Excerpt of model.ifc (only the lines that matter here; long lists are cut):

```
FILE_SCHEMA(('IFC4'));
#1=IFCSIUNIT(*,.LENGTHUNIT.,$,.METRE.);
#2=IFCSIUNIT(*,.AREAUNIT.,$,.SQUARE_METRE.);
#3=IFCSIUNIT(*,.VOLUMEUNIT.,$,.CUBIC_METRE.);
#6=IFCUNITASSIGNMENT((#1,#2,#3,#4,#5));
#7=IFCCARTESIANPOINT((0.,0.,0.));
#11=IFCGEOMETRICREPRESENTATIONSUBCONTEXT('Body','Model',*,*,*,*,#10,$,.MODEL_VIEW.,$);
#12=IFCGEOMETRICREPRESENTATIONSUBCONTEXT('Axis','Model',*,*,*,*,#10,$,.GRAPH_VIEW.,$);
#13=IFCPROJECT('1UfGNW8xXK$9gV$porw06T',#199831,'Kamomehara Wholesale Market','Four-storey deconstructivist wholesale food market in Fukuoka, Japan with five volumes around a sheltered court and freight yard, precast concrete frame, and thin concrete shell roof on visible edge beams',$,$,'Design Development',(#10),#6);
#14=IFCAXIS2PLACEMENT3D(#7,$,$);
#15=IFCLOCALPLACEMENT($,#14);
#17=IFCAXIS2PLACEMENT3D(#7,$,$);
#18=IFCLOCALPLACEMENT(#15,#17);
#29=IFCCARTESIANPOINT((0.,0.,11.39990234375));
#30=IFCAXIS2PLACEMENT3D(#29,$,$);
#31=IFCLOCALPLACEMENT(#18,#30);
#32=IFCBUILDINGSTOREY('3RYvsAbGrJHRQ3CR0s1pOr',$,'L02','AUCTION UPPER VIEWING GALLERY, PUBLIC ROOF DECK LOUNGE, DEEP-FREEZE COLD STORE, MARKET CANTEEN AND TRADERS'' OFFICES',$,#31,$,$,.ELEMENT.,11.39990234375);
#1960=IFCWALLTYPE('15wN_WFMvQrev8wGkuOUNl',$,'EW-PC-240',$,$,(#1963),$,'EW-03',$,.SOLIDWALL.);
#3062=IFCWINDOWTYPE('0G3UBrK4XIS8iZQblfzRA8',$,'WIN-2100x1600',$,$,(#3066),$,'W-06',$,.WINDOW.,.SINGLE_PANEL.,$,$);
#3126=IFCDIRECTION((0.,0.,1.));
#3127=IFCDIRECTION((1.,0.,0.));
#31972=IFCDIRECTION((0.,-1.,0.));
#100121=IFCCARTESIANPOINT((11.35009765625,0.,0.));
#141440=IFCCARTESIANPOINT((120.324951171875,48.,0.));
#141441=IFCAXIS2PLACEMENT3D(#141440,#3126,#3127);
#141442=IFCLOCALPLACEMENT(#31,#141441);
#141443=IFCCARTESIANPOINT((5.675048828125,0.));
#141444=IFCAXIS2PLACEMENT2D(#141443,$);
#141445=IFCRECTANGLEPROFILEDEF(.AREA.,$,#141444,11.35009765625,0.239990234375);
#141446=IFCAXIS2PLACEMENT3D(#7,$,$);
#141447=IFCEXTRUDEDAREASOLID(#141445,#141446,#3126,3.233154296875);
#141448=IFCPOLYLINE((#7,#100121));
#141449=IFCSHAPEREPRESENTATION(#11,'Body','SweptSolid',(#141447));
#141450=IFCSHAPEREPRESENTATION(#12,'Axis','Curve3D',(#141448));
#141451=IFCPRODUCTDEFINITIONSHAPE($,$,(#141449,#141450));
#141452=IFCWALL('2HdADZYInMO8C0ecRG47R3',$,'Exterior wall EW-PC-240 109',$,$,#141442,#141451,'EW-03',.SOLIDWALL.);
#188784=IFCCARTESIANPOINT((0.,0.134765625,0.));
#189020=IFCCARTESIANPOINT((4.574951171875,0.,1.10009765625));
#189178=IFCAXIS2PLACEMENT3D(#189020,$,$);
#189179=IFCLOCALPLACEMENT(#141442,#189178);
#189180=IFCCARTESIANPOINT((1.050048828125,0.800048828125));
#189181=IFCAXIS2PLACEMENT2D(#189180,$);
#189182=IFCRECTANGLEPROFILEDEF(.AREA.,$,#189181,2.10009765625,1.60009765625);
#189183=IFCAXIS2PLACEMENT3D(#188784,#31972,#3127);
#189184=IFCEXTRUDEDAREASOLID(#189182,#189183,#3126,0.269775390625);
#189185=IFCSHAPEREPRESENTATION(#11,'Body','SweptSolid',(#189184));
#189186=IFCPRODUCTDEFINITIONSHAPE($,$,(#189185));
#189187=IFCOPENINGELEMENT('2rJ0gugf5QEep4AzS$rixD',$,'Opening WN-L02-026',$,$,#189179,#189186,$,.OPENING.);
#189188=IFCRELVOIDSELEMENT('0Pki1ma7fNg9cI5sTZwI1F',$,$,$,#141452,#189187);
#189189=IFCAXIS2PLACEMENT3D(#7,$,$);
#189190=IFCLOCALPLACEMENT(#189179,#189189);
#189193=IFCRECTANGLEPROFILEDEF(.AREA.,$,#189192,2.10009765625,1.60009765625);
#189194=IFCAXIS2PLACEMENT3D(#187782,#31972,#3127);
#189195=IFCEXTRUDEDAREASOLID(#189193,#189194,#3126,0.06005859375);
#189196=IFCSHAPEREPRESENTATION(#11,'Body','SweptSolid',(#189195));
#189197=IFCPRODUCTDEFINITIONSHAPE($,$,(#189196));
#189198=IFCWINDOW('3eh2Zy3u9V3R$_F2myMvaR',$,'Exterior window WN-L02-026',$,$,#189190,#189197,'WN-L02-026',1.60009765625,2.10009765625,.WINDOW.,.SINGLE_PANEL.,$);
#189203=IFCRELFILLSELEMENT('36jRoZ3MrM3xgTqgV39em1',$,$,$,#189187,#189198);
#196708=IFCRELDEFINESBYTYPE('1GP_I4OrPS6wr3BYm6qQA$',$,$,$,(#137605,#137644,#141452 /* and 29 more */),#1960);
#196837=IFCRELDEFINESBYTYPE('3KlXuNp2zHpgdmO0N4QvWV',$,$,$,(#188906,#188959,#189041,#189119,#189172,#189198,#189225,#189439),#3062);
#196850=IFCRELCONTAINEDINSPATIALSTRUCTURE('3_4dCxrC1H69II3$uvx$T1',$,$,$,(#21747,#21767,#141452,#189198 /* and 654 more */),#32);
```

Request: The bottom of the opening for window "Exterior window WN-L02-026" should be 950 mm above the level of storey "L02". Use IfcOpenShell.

```python
import numpy as np
import ifcopenshell
import ifcopenshell.api.geometry
import ifcopenshell.geom
import ifcopenshell.util.element
import ifcopenshell.util.placement
import ifcopenshell.util.shape
import ifcopenshell.util.unit

model = ifcopenshell.open("model.ifc")
unit_scale = ifcopenshell.util.unit.calculate_unit_scale(model)

window = model.by_guid("3eh2Zy3u9V3R$_F2myMvaR")
opening = window.FillsVoids[0].RelatingOpeningElement
storey = ifcopenshell.util.element.get_container(window, ifc_class="IfcBuildingStorey")
level = ifcopenshell.util.placement.get_local_placement(storey.ObjectPlacement)[2, 3]

# The opening's origin need not be at the sill, so measure its lowest point.
shape = ifcopenshell.geom.create_shape(ifcopenshell.geom.settings(), opening)
bottom = ifcopenshell.util.shape.get_shape_bottom_elevation(shape, shape.geometry) / unit_scale
dz = level + 0.95 - bottom

shift = np.array([0.0, 0.0, dz])
# The window is placed relative to its opening, so it follows when the opening moves.
matrix = ifcopenshell.util.placement.get_local_placement(opening.ObjectPlacement)
matrix[:3, 3] += shift
ifcopenshell.api.geometry.edit_object_placement(
    model, product=opening, matrix=matrix, is_si=False, should_transform_children=True
)

print(f"moved by {dz * unit_scale:+.3f} m")

model.write("model_v2.ifc")
```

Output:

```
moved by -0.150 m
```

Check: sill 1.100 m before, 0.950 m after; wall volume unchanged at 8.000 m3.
